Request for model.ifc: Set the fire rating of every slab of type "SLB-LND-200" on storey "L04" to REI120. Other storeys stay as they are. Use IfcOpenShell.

First a look at what the model holds.

```python
import ifcopenshell
import ifcopenshell.util.element

model = ifcopenshell.open("model.ifc")
print(model.schema)
storey = next(s for s in model.by_type("IfcBuildingStorey") if s.Name == "L04")
slabs = [e for e in ifcopenshell.util.element.get_decomposition(storey) if e.is_a("IfcSlab")]
seen = {}
for e in slabs:
    element_type = ifcopenshell.util.element.get_type(e)
    key = (element_type.Name if element_type != e and element_type else None, ifcopenshell.util.element.get_pset(e, "Pset_SlabCommon", "FireRating"))
    seen[key] = seen.get(key, 0) + 1
for (name, value), count in sorted(seen.items(), key=str):
    print(count, "x", name, "|", value)
```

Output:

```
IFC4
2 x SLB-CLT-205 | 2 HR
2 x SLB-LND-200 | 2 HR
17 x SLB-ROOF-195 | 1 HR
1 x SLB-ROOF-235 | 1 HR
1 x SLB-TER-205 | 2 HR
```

```python
import ifcopenshell
import ifcopenshell.api.pset
import ifcopenshell.util.element

model = ifcopenshell.open("model.ifc")

storey = next(s for s in model.by_type("IfcBuildingStorey") if s.Name == "L04")
slabs = [e for e in ifcopenshell.util.element.get_decomposition(storey) if e.is_a("IfcSlab")]

count = 0
for e in slabs:
    element_type = ifcopenshell.util.element.get_type(e)
    if element_type in (None, e) or element_type.Name != "SLB-LND-200":
        continue
    # add_pset returns the element's existing set when there is one.
    pset = ifcopenshell.api.pset.add_pset(model, product=e, name="Pset_SlabCommon")
    ifcopenshell.api.pset.edit_pset(model, pset=pset, properties={"FireRating": "REI120"})
    count += 1

print(count, "slabs updated")

model.write("model_rev.ifc")
```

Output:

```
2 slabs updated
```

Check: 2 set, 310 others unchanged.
